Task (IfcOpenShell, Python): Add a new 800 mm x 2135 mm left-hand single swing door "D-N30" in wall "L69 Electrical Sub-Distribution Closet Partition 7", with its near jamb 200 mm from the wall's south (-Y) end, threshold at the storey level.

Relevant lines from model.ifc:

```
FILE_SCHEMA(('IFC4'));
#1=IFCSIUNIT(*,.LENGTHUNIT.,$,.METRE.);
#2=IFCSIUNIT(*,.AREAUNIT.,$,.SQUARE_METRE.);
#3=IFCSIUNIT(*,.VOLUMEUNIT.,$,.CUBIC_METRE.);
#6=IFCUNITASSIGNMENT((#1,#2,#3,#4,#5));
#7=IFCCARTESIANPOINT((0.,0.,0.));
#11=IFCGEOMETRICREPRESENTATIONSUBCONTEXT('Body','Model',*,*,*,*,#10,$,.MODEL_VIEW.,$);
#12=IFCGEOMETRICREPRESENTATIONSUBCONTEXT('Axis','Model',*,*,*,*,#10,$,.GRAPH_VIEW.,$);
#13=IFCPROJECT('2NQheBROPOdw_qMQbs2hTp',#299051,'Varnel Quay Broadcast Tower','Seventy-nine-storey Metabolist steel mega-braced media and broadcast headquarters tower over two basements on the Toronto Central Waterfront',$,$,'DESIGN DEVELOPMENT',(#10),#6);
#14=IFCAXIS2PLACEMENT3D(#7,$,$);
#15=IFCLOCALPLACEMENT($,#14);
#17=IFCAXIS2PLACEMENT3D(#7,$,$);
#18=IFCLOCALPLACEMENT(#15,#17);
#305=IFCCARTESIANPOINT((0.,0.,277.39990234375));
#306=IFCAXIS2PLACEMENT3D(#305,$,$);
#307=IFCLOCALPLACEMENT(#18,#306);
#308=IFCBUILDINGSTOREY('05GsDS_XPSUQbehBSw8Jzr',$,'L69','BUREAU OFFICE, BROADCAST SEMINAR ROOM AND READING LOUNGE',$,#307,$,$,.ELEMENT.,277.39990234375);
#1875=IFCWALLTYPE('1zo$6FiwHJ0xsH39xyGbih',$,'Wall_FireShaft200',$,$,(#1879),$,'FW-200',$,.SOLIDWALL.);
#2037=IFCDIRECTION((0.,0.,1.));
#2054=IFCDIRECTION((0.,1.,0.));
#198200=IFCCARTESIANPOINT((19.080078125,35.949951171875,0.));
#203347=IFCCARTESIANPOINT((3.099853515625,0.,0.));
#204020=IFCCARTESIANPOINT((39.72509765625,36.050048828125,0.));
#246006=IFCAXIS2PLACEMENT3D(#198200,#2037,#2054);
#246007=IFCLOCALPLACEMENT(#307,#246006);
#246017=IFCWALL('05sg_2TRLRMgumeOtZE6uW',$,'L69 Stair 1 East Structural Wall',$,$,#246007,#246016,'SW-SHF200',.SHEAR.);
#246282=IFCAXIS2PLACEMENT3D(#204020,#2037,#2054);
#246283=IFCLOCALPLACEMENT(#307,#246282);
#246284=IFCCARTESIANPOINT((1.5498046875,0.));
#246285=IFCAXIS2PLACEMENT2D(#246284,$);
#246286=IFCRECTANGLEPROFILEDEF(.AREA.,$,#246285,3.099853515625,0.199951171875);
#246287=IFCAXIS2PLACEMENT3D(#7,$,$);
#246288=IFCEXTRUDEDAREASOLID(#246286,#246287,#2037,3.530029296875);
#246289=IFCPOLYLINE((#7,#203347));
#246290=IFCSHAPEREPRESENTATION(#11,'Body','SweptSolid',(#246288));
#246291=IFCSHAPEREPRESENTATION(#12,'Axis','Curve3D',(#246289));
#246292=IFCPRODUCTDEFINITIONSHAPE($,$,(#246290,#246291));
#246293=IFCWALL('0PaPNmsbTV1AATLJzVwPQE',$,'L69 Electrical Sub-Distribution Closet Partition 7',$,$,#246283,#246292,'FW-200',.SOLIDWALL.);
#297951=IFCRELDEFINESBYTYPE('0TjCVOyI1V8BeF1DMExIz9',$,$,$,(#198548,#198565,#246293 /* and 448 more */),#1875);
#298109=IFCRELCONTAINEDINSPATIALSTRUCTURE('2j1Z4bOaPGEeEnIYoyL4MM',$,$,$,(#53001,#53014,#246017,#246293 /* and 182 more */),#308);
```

```python
import numpy as np
import ifcopenshell
import ifcopenshell.api.feature
import ifcopenshell.api.geometry
import ifcopenshell.api.root
import ifcopenshell.api.spatial
import ifcopenshell.geom
import ifcopenshell.util.element
import ifcopenshell.util.placement
import ifcopenshell.util.representation
import ifcopenshell.util.shape
import ifcopenshell.util.unit

model = ifcopenshell.open("model.ifc")
unit_scale = ifcopenshell.util.unit.calculate_unit_scale(model)
settings = ifcopenshell.geom.settings()


def volume(element):
    """Net volume in cubic metres, openings subtracted."""
    shape = ifcopenshell.geom.create_shape(settings, element)
    return ifcopenshell.util.shape.get_volume(shape.geometry)


wall = model.by_guid("0PaPNmsbTV1AATLJzVwPQE")
storey = ifcopenshell.util.element.get_container(wall, ifc_class="IfcBuildingStorey")
context = ifcopenshell.util.representation.get_context(model, "Model", "Body", "MODEL_VIEW")
before = volume(wall)

width, height, from_end, sill = 0.8, 2.135, 0.2, 0.0  # metres

# The wall runs along its own X axis, and the end named is its -X end.
wall_shape = ifcopenshell.geom.create_shape(settings, wall)
x, y, z = ifcopenshell.util.shape.get_vertices(wall_shape.geometry).T
start = x.min() + from_end
face, thickness = float(y.min()), float(y.max() - y.min())
wall_matrix = ifcopenshell.util.placement.get_local_placement(wall.ObjectPlacement)
level = ifcopenshell.util.placement.get_local_placement(storey.ObjectPlacement)[2, 3]


def in_wall(x, y):
    """Placement at x, y metres in the wall's axes, at sill height."""
    matrix = wall_matrix.copy()
    matrix[:, 3] = wall_matrix @ np.array([x / unit_scale, y / unit_scale, 0.0, 1.0])
    matrix[2, 3] = level + sill / unit_scale
    return matrix


# Opening: a box that overshoots both wall faces by 50 mm.
opening = ifcopenshell.api.root.create_entity(model, ifc_class="IfcOpeningElement", predefined_type="OPENING")
box = ifcopenshell.api.geometry.add_wall_representation(
    model, context=context, length=width, height=height, thickness=thickness + 0.1
)
ifcopenshell.api.geometry.assign_representation(model, product=opening, representation=box)
ifcopenshell.api.geometry.edit_object_placement(model, product=opening, matrix=in_wall(start, face - 0.05), is_si=False)
ifcopenshell.api.feature.add_feature(model, feature=opening, element=wall)

door = ifcopenshell.api.root.create_entity(model, ifc_class="IfcDoor", name="D-N30", predefined_type="DOOR")
door.OverallWidth, door.OverallHeight = width / unit_scale, height / unit_scale
door.OperationType = "SINGLE_SWING_LEFT"
body = ifcopenshell.api.geometry.add_door_representation(
    model,
    context=context,
    overall_width=door.OverallWidth,
    overall_height=door.OverallHeight,
    operation_type="SINGLE_SWING_LEFT",
    lining_properties={"LiningDepth": thickness / unit_scale, "ThresholdDepth": thickness / unit_scale},
)
ifcopenshell.api.geometry.assign_representation(model, product=door, representation=body)
ifcopenshell.api.spatial.assign_container(model, products=[door], relating_structure=storey)
ifcopenshell.api.feature.add_filling(model, opening=opening, element=door)

# The lining spans the wall, so the door starts at the wall face.
ifcopenshell.api.geometry.edit_object_placement(model, product=door, matrix=in_wall(start, face), is_si=False)

after = volume(wall)

print(f"wall volume {before:.3f} -> {after:.3f} m3")

model.write("model-out.ifc")
```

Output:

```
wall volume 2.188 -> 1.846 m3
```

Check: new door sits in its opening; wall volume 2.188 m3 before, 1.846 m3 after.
